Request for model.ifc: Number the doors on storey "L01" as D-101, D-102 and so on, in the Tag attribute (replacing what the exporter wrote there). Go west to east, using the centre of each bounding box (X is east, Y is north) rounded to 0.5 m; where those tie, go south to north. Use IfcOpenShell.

First a look at what the model holds.

```python
import ifcopenshell
import ifcopenshell.util.element
import ifcopenshell.util.placement

model = ifcopenshell.open("model.ifc")
print(model.schema)
storey = next(s for s in model.by_type("IfcBuildingStorey") if s.Name == "L01")
doors = [e for e in ifcopenshell.util.element.get_decomposition(storey) if e.is_a("IfcDoor")]
for e in sorted(doors, key=lambda e: e.id()):
    origin = ifcopenshell.util.placement.get_local_placement(e.ObjectPlacement)[:3, 3]
    print(e.id(), e.Tag, e.Name, origin.round(2) + 0.0, sep=" | ")
```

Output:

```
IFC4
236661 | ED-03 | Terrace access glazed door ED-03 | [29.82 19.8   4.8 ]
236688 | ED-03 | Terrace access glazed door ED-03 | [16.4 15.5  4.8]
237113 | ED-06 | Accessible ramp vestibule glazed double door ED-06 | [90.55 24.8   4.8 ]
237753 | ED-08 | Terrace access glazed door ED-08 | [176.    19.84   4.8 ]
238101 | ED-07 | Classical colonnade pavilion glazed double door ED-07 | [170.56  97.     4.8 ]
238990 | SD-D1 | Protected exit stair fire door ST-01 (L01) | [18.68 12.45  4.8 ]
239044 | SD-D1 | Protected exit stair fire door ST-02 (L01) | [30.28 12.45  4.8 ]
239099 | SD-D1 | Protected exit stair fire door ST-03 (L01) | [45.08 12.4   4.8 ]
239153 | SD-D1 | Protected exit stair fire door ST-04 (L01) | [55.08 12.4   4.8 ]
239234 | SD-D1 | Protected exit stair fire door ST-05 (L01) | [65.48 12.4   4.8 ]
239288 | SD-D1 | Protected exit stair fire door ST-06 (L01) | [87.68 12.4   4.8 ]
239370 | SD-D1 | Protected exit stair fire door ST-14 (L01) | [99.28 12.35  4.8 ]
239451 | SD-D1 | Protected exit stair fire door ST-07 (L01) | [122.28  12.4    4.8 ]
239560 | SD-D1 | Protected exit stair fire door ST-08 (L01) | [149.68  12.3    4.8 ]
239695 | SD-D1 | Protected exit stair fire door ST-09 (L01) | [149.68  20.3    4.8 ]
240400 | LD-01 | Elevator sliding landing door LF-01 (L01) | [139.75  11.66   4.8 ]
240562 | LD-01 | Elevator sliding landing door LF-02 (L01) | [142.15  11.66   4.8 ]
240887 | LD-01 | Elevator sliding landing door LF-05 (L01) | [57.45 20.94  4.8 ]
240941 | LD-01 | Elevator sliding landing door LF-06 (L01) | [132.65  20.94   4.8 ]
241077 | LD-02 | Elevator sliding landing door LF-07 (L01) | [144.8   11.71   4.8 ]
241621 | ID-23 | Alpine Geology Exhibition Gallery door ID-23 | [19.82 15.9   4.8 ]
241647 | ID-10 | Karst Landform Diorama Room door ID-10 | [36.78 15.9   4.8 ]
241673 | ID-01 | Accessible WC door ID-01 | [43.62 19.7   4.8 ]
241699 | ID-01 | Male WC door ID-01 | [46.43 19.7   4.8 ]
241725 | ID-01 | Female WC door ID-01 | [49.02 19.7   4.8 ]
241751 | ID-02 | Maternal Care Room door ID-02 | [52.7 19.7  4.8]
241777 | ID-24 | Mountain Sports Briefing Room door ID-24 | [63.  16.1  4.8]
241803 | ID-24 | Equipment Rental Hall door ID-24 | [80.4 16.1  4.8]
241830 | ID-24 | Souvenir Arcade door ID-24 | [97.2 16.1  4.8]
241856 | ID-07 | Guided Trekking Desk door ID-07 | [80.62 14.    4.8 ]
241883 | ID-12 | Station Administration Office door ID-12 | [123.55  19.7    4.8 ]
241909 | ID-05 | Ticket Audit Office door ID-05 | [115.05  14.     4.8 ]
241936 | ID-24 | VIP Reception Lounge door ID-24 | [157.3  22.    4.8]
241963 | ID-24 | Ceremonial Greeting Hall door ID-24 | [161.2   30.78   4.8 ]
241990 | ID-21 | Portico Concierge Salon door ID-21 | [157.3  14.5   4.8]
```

```python
import ifcopenshell
import ifcopenshell.geom
import ifcopenshell.util.element
import ifcopenshell.util.shape

model = ifcopenshell.open("model.ifc")
settings = ifcopenshell.geom.settings()
settings.set("use-world-coords", True)


def centre(element):
    shape = ifcopenshell.geom.create_shape(settings, element)
    return ifcopenshell.util.shape.get_bbox_centroid(shape.geometry)


storey = next(s for s in model.by_type("IfcBuildingStorey") if s.Name == "L01")
doors = [e for e in ifcopenshell.util.element.get_decomposition(storey) if e.is_a("IfcDoor")]

# Insertion points can sit at a corner or the storey origin, so sort by the geometry (in metres).
centres = {e: centre(e) for e in doors}
doors.sort(key=lambda e: (round(centres[e][0] / 0.5), centres[e][1]))

for i, e in enumerate(doors, start=1):
    number = f"D-1{i:02d}"
    e.Tag = number
    print(e.id(), number)

model.write("model_updated.ifc")
```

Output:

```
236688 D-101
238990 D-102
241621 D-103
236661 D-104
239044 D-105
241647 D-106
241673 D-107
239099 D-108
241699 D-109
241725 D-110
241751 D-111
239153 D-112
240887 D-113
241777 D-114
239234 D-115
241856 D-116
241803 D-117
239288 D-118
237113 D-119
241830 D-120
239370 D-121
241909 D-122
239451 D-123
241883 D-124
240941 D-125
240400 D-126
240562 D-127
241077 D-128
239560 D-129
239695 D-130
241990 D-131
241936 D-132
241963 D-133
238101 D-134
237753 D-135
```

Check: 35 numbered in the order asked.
